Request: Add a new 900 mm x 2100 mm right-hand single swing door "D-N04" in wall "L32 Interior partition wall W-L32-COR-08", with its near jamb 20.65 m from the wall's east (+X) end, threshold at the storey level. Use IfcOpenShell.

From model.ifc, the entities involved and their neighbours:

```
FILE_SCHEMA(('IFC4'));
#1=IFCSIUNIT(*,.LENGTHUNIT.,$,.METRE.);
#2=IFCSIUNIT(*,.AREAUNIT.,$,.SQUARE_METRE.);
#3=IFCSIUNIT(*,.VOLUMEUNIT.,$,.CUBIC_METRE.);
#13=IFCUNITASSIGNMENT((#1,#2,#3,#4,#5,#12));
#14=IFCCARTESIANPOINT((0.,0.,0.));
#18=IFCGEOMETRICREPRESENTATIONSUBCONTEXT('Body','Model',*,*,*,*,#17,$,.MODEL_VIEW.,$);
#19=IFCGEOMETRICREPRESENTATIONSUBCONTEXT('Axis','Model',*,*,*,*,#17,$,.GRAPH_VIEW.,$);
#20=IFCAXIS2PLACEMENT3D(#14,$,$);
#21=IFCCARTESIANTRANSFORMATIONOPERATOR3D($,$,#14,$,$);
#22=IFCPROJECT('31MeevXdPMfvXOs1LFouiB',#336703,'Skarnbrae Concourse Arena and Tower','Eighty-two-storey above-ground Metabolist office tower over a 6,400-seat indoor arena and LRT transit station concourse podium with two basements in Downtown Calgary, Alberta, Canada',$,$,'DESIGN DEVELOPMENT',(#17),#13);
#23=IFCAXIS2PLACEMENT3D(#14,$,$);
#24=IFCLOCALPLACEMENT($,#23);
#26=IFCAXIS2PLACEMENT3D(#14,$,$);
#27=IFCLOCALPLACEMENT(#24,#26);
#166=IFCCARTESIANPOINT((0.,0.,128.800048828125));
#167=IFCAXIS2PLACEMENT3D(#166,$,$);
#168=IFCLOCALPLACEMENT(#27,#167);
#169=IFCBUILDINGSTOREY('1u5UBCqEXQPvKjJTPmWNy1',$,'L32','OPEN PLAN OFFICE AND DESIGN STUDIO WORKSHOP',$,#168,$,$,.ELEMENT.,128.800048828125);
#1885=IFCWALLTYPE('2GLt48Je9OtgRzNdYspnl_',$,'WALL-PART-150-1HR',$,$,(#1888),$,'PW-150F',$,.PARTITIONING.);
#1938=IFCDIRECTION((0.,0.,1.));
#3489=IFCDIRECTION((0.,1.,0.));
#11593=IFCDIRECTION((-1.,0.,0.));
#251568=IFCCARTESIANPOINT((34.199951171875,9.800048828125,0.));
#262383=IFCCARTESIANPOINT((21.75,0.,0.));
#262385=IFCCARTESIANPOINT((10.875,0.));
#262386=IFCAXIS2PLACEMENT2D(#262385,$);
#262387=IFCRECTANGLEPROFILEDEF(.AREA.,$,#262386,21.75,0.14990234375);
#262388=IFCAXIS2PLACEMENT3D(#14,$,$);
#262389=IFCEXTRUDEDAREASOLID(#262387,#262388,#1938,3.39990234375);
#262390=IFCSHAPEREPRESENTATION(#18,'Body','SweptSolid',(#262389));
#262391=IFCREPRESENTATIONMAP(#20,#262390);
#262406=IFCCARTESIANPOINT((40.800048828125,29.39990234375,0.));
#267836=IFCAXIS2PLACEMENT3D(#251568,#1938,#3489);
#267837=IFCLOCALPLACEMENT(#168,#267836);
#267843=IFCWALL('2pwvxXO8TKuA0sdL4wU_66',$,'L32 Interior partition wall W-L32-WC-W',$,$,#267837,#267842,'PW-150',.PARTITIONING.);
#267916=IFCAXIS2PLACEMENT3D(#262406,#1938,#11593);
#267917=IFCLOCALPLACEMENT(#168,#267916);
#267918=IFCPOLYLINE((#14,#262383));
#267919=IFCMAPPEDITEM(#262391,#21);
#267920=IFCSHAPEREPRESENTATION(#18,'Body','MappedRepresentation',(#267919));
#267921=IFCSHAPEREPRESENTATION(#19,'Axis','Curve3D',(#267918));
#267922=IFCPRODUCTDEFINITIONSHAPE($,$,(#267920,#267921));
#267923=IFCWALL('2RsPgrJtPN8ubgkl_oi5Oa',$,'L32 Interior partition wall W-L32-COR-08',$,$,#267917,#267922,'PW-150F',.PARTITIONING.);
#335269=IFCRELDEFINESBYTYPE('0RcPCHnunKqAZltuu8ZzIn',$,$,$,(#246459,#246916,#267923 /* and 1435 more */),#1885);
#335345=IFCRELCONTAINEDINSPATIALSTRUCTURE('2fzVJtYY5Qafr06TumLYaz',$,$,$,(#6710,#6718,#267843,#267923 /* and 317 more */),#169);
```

```python
import numpy as np
import ifcopenshell
import ifcopenshell.api.feature
import ifcopenshell.api.geometry
import ifcopenshell.api.root
import ifcopenshell.api.spatial
import ifcopenshell.geom
import ifcopenshell.util.element
import ifcopenshell.util.placement
import ifcopenshell.util.representation
import ifcopenshell.util.shape
import ifcopenshell.util.unit

model = ifcopenshell.open("model.ifc")
unit_scale = ifcopenshell.util.unit.calculate_unit_scale(model)
settings = ifcopenshell.geom.settings()


def volume(element):
    """Net volume in cubic metres, openings subtracted."""
    shape = ifcopenshell.geom.create_shape(settings, element)
    return ifcopenshell.util.shape.get_volume(shape.geometry)


wall = model.by_guid("2RsPgrJtPN8ubgkl_oi5Oa")
storey = ifcopenshell.util.element.get_container(wall, ifc_class="IfcBuildingStorey")
context = ifcopenshell.util.representation.get_context(model, "Model", "Body", "MODEL_VIEW")
before = volume(wall)

width, height, from_end, sill = 0.9, 2.1, 20.65, 0.0  # metres

# The wall runs along its own X axis, and the end named is its -X end.
wall_shape = ifcopenshell.geom.create_shape(settings, wall)
x, y, z = ifcopenshell.util.shape.get_vertices(wall_shape.geometry).T
start = x.min() + from_end
face, thickness = float(y.min()), float(y.max() - y.min())
wall_matrix = ifcopenshell.util.placement.get_local_placement(wall.ObjectPlacement)
level = ifcopenshell.util.placement.get_local_placement(storey.ObjectPlacement)[2, 3]


def in_wall(x, y):
    """Placement at x, y metres in the wall's axes, at sill height."""
    matrix = wall_matrix.copy()
    matrix[:, 3] = wall_matrix @ np.array([x / unit_scale, y / unit_scale, 0.0, 1.0])
    matrix[2, 3] = level + sill / unit_scale
    return matrix


# Opening: a box that overshoots both wall faces by 50 mm.
opening = ifcopenshell.api.root.create_entity(model, ifc_class="IfcOpeningElement", predefined_type="OPENING")
box = ifcopenshell.api.geometry.add_wall_representation(
    model, context=context, length=width, height=height, thickness=thickness + 0.1
)
ifcopenshell.api.geometry.assign_representation(model, product=opening, representation=box)
ifcopenshell.api.geometry.edit_object_placement(model, product=opening, matrix=in_wall(start, face - 0.05), is_si=False)
ifcopenshell.api.feature.add_feature(model, feature=opening, element=wall)

door = ifcopenshell.api.root.create_entity(model, ifc_class="IfcDoor", name="D-N04", predefined_type="DOOR")
door.OverallWidth, door.OverallHeight = width / unit_scale, height / unit_scale
door.OperationType = "SINGLE_SWING_RIGHT"
body = ifcopenshell.api.geometry.add_door_representation(
    model,
    context=context,
    overall_width=door.OverallWidth,
    overall_height=door.OverallHeight,
    operation_type="SINGLE_SWING_RIGHT",
    lining_properties={"LiningDepth": thickness / unit_scale, "ThresholdDepth": thickness / unit_scale},
)
ifcopenshell.api.geometry.assign_representation(model, product=door, representation=body)
ifcopenshell.api.spatial.assign_container(model, products=[door], relating_structure=storey)
ifcopenshell.api.feature.add_filling(model, opening=opening, element=door)

# The lining spans the wall, so the door starts at the wall face.
ifcopenshell.api.geometry.edit_object_placement(model, product=door, matrix=in_wall(start, face), is_si=False)

after = volume(wall)

print(f"wall volume {before:.3f} -> {after:.3f} m3")

model.write("model_edited.ifc")
```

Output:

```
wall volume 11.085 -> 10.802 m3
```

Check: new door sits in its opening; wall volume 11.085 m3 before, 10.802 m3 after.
